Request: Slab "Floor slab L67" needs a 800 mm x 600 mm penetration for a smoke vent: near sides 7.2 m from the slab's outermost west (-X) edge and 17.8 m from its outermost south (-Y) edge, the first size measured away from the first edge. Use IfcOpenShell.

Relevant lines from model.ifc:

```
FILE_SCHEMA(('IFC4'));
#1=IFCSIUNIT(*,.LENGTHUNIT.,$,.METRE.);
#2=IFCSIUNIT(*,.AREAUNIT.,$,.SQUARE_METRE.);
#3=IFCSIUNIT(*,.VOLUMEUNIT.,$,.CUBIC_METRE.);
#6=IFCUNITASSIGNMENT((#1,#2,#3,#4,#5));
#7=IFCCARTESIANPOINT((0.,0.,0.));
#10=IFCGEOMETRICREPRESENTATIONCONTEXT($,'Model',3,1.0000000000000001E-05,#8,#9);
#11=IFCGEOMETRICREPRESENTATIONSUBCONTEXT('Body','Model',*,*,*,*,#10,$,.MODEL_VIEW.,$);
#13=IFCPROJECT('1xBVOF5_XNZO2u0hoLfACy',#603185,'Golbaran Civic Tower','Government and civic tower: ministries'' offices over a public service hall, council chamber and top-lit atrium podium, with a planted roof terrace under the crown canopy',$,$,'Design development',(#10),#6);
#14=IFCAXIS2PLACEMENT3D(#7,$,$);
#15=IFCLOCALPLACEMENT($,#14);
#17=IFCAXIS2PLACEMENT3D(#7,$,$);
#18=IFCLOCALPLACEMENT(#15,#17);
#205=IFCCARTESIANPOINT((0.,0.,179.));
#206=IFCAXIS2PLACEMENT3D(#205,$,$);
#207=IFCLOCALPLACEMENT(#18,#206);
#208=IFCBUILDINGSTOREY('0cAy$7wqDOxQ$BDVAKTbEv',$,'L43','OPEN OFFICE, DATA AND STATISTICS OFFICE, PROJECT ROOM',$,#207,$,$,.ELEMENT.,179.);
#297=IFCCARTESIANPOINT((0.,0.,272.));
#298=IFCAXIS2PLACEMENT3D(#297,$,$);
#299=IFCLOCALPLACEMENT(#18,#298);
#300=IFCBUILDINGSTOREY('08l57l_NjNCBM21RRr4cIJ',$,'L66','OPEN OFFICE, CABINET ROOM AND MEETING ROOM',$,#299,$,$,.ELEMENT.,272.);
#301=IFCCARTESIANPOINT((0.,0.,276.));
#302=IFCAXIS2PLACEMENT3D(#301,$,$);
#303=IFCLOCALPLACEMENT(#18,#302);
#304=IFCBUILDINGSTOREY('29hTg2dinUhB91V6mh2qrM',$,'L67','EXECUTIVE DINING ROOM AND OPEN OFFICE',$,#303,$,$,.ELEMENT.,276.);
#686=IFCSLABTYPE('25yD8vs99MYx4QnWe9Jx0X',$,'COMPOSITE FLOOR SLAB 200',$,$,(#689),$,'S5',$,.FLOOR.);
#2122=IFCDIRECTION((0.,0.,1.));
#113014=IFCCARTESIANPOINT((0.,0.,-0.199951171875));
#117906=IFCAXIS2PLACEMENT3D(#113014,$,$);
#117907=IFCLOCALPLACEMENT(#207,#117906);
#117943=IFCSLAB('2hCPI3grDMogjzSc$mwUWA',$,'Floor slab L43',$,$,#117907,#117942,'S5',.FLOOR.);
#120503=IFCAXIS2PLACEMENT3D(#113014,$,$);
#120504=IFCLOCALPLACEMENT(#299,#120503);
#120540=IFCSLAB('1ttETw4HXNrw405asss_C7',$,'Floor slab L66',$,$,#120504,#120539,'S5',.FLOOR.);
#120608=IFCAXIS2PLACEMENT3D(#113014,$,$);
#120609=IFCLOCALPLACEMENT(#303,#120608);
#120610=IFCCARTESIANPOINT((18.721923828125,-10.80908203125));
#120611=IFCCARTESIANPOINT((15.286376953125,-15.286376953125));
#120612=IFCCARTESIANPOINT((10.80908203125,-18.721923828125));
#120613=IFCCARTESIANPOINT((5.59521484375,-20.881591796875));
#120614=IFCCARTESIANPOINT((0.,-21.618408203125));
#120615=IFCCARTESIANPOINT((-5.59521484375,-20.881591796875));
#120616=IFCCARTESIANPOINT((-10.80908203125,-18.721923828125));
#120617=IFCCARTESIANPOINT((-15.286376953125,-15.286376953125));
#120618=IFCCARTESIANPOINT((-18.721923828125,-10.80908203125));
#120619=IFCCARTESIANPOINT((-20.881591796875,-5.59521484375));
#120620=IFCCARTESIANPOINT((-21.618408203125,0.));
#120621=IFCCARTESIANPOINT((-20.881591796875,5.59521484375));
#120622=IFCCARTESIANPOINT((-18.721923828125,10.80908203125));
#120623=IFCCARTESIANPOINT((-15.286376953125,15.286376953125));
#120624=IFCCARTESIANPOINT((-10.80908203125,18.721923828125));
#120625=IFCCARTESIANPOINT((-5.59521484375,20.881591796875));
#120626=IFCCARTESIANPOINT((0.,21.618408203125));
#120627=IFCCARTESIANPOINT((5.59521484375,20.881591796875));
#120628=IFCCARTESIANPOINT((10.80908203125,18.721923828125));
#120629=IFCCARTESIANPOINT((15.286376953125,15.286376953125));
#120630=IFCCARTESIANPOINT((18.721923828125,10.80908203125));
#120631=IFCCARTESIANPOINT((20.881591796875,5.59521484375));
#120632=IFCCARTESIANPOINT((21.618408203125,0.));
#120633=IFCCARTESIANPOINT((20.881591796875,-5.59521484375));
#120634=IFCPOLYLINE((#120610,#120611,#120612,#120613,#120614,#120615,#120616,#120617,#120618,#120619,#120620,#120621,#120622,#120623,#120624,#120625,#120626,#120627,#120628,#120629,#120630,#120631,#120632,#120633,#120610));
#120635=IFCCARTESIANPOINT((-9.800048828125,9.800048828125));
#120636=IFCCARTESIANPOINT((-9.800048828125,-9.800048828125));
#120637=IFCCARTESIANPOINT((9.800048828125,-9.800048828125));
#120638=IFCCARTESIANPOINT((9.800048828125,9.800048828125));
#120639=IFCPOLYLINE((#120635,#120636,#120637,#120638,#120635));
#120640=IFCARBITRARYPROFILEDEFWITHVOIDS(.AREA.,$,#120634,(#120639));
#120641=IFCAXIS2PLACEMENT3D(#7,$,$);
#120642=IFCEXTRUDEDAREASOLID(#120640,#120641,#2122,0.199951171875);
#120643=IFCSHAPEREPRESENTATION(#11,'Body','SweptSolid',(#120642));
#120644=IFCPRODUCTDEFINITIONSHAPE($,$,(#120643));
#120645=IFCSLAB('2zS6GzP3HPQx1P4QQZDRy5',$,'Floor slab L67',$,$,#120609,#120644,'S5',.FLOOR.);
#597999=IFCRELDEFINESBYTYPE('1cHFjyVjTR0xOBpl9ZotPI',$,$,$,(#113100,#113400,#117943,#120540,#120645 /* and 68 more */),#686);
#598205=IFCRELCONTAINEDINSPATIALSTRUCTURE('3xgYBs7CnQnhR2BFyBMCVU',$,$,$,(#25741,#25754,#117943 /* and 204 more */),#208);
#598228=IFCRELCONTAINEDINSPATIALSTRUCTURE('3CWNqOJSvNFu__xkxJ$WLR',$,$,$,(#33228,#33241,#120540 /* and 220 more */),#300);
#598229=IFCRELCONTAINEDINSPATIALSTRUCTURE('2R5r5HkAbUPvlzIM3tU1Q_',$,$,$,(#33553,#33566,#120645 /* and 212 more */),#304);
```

```python
import numpy as np
import ifcopenshell
import ifcopenshell.api.feature
import ifcopenshell.api.geometry
import ifcopenshell.api.root
import ifcopenshell.geom
import ifcopenshell.util.placement
import ifcopenshell.util.representation
import ifcopenshell.util.shape
import ifcopenshell.util.unit

model = ifcopenshell.open("model.ifc")
unit_scale = ifcopenshell.util.unit.calculate_unit_scale(model)
settings = ifcopenshell.geom.settings()


def volume(element):
    """Net volume in cubic metres, openings subtracted."""
    shape = ifcopenshell.geom.create_shape(settings, element)
    return ifcopenshell.util.shape.get_volume(shape.geometry)


slab = model.by_id(120645)
before = volume(slab)

# Extent in the slab's own axes, in metres. The edges named are its -X and -Y sides.
slab_shape = ifcopenshell.geom.create_shape(settings, slab)
vertices = ifcopenshell.util.shape.get_vertices(slab_shape.geometry)
x_min, y_min, bottom = vertices.min(axis=0)
top = vertices[:, 2].max()

opening = ifcopenshell.api.root.create_entity(model, ifc_class="IfcOpeningElement", name="Smoke vent opening", predefined_type="OPENING")
context = ifcopenshell.util.representation.get_context(model, "Model", "Body", "MODEL_VIEW")
width, depth = 0.8, 0.6
outline = [(0.0, 0.0), (width, 0.0), (width, depth), (0.0, depth), (0.0, 0.0)]
# Overshoot both faces by 50 mm so the cut is clean.
shape = ifcopenshell.api.geometry.add_slab_representation(
    model, context=context, depth=top - bottom + 0.1, polyline=outline
)
ifcopenshell.api.geometry.assign_representation(model, product=opening, representation=shape)

matrix = ifcopenshell.util.placement.get_local_placement(slab.ObjectPlacement)
matrix[:, 3] = matrix @ np.append(np.array([x_min + 7.2, y_min + 17.8, bottom - 0.05]) / unit_scale, 1.0)
ifcopenshell.api.geometry.edit_object_placement(model, product=opening, matrix=matrix, is_si=False)
ifcopenshell.api.feature.add_feature(model, feature=opening, element=slab)

after = volume(slab)

print(f"slab volume {before:.3f} -> {after:.3f} m3")

model.write("model_edited.ifc")
```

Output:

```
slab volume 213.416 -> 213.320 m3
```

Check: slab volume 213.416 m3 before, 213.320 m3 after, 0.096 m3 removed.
